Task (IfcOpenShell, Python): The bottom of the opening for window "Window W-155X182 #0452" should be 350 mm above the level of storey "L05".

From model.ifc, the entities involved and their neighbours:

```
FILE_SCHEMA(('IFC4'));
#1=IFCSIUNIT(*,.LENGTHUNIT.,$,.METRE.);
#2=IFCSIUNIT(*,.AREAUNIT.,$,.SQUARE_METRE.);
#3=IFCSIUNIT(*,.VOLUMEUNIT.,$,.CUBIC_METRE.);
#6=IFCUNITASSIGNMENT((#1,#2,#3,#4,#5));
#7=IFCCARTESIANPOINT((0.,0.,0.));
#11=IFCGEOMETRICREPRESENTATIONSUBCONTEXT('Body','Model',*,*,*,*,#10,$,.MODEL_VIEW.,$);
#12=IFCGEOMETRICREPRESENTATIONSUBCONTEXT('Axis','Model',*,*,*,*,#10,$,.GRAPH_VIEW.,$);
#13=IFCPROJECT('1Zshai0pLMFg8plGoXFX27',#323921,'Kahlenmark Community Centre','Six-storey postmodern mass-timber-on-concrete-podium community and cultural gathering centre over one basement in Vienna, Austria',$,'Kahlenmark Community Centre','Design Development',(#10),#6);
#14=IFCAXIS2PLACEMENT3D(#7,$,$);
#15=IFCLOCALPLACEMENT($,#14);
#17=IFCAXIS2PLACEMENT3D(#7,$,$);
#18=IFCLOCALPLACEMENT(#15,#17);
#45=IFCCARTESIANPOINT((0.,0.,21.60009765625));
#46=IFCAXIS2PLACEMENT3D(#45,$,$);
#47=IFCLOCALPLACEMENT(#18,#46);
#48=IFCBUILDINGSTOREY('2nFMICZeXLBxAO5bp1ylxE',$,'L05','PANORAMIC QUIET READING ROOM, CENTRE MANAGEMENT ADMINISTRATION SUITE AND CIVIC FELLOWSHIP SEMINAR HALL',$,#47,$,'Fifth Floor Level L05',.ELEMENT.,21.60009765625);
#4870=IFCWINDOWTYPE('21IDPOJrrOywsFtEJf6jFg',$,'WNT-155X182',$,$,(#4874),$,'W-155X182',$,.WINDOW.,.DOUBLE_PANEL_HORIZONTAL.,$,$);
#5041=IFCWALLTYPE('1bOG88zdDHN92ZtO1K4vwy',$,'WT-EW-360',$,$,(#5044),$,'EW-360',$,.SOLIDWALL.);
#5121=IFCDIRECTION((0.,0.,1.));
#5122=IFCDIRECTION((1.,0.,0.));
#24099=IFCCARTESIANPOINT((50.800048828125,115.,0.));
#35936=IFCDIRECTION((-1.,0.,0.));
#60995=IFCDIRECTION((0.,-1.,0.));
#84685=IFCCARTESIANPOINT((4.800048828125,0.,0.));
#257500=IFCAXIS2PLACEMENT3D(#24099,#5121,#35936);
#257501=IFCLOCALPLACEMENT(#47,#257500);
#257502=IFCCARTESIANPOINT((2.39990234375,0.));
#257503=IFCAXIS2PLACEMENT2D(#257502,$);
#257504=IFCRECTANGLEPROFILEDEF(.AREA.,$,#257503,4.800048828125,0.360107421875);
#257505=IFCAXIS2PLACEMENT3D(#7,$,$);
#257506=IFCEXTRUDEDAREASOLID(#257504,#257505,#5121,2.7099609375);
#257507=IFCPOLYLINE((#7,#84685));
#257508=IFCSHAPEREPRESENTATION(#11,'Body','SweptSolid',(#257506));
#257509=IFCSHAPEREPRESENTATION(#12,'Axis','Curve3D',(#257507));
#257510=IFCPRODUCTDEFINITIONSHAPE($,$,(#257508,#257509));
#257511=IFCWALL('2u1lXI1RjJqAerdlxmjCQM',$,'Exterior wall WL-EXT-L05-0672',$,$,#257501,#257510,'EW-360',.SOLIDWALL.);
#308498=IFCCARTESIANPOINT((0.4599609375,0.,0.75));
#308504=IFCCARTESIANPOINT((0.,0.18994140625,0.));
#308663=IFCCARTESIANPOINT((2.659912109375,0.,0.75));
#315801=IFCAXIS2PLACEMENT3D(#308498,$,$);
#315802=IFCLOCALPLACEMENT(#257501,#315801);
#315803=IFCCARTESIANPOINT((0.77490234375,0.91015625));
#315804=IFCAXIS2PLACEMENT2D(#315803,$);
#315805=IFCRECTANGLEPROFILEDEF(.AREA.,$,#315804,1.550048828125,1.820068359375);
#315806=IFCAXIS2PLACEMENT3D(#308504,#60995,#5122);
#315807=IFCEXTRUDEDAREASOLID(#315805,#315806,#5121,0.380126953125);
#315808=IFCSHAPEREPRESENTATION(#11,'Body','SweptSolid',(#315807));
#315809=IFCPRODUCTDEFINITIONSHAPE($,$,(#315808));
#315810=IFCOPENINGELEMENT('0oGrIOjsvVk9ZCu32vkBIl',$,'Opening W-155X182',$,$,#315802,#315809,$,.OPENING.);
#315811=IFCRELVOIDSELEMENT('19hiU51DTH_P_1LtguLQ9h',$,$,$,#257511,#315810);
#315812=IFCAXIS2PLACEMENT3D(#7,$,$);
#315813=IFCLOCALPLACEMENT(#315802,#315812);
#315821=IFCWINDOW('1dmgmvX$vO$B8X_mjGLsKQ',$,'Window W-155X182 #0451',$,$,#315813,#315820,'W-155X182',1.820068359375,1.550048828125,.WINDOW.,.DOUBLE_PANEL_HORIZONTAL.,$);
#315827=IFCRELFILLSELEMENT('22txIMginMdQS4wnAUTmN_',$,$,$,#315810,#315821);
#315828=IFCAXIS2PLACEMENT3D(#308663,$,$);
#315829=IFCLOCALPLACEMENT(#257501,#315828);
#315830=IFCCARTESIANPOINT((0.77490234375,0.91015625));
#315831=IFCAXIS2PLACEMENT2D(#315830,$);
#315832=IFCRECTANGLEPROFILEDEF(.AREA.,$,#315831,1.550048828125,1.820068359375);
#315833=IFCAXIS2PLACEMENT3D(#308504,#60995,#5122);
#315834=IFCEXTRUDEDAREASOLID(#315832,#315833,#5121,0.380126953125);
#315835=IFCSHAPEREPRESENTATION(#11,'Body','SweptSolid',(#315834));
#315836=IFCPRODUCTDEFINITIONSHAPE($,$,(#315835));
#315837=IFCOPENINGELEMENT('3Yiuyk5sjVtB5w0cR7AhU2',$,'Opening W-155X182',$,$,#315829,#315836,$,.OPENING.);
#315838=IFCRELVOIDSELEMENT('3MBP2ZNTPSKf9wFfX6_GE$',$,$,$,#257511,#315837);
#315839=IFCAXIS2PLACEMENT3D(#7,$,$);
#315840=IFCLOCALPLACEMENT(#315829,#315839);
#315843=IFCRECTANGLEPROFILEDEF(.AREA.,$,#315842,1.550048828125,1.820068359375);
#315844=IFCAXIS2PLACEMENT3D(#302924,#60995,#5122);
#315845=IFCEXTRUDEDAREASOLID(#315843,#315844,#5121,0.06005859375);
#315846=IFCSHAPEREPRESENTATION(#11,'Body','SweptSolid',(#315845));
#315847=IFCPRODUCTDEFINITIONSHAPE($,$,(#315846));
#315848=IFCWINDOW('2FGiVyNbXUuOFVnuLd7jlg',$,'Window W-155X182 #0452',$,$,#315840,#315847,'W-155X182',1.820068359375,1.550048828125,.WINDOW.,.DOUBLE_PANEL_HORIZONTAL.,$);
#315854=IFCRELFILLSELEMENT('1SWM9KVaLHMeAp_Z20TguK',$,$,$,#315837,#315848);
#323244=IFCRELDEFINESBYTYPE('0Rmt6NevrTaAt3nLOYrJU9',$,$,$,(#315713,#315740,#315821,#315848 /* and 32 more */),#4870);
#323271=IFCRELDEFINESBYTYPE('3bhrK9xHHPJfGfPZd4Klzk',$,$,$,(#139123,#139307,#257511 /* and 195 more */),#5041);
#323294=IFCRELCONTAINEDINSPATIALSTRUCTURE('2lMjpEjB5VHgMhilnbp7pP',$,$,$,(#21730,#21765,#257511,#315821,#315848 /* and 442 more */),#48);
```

```python
import numpy as np
import ifcopenshell
import ifcopenshell.api.geometry
import ifcopenshell.geom
import ifcopenshell.util.element
import ifcopenshell.util.placement
import ifcopenshell.util.shape
import ifcopenshell.util.unit

model = ifcopenshell.open("model.ifc")
unit_scale = ifcopenshell.util.unit.calculate_unit_scale(model)

window = model.by_guid("2FGiVyNbXUuOFVnuLd7jlg")
opening = window.FillsVoids[0].RelatingOpeningElement
storey = ifcopenshell.util.element.get_container(window, ifc_class="IfcBuildingStorey")
level = ifcopenshell.util.placement.get_local_placement(storey.ObjectPlacement)[2, 3]

# The opening's origin need not be at the sill, so measure its lowest point.
shape = ifcopenshell.geom.create_shape(ifcopenshell.geom.settings(), opening)
bottom = ifcopenshell.util.shape.get_shape_bottom_elevation(shape, shape.geometry) / unit_scale
dz = level + 0.35 - bottom

shift = np.array([0.0, 0.0, dz])
# The window is placed relative to its opening, so it follows when the opening moves.
matrix = ifcopenshell.util.placement.get_local_placement(opening.ObjectPlacement)
matrix[:3, 3] += shift
ifcopenshell.api.geometry.edit_object_placement(
    model, product=opening, matrix=matrix, is_si=False, should_transform_children=True
)

print(f"moved by {dz * unit_scale:+.3f} m")

model.write("model_updated.ifc")
```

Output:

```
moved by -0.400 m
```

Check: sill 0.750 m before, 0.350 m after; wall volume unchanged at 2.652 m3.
